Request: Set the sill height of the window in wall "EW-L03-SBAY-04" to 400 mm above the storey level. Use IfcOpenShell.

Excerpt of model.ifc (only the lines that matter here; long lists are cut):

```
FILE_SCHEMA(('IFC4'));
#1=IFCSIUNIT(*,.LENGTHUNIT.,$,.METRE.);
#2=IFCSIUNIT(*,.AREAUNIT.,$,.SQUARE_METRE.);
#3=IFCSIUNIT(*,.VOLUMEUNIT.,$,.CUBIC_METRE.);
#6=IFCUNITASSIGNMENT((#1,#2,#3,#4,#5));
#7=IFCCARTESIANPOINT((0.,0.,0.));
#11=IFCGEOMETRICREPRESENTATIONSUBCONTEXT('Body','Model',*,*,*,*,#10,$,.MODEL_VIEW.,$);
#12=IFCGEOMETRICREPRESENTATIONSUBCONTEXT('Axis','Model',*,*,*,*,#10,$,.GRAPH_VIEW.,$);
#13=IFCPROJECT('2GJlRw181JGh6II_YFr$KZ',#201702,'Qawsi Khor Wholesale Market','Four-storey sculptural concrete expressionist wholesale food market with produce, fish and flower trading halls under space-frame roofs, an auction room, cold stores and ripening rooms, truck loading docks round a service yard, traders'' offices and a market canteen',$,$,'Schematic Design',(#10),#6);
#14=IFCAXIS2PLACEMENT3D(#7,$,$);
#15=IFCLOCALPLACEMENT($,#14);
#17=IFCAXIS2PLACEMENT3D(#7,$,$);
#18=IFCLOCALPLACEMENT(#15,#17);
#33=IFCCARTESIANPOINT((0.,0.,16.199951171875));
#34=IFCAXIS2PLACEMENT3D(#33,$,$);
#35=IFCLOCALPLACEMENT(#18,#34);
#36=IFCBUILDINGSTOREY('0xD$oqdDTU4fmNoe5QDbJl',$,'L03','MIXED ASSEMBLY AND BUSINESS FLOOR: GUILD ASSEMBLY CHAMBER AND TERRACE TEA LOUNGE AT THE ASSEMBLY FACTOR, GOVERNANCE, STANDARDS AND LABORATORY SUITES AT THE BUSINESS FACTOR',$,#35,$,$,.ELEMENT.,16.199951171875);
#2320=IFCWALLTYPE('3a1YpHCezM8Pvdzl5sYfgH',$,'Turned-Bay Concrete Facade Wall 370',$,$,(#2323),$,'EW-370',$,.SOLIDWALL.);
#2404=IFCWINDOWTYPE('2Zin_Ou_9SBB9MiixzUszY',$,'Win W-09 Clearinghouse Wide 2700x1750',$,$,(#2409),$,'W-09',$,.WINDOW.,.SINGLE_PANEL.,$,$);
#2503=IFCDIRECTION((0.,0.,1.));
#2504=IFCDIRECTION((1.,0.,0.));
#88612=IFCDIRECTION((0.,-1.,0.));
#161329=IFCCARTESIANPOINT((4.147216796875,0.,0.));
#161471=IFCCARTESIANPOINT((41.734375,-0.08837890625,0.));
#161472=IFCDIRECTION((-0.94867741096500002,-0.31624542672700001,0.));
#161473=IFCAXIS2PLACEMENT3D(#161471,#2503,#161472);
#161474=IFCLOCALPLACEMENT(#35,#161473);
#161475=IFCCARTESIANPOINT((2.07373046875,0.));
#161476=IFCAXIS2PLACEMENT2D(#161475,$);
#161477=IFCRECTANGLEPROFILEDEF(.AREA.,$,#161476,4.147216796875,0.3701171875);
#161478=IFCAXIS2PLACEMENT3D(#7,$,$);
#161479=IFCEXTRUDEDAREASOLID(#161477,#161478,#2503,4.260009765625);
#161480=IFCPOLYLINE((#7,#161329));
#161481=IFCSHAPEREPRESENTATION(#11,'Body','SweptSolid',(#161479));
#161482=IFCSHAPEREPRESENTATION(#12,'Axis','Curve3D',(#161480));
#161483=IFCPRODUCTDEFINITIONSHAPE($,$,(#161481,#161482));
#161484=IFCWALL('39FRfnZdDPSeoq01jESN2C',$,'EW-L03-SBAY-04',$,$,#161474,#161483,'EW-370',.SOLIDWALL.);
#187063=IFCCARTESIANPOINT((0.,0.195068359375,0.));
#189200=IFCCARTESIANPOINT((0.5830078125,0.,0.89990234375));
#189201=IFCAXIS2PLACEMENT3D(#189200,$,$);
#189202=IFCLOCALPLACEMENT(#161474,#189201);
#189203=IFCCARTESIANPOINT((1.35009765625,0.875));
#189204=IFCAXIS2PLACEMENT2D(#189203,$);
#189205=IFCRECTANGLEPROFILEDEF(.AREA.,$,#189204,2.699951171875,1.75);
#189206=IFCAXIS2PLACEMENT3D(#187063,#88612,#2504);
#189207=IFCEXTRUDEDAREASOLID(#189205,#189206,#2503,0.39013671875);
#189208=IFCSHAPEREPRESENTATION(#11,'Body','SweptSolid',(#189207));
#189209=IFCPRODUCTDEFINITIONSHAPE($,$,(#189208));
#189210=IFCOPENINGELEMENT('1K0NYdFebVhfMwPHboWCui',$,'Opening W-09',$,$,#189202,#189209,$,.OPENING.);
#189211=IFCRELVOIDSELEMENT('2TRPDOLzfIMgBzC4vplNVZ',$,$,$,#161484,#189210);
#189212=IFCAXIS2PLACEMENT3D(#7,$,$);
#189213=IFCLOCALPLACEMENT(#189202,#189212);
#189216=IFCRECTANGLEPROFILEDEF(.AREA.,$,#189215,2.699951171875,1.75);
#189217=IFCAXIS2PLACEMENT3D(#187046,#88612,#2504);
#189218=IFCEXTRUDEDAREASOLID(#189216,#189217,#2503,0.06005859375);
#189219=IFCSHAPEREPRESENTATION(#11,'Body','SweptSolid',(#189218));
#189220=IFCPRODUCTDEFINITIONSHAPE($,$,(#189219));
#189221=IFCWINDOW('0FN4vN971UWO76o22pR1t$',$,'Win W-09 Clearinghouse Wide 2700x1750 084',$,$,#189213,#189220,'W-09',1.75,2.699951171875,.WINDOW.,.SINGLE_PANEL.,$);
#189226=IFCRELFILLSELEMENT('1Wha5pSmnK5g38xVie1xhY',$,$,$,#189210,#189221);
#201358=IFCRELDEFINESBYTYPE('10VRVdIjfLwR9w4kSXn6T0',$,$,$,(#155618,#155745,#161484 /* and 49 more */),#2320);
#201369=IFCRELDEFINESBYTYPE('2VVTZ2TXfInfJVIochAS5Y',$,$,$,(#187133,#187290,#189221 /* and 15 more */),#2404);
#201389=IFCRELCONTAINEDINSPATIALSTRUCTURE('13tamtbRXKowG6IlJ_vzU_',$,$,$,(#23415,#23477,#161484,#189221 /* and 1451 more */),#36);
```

```python
import numpy as np
import ifcopenshell
import ifcopenshell.api.geometry
import ifcopenshell.geom
import ifcopenshell.util.element
import ifcopenshell.util.placement
import ifcopenshell.util.shape
import ifcopenshell.util.unit

model = ifcopenshell.open("model.ifc")
unit_scale = ifcopenshell.util.unit.calculate_unit_scale(model)

window = model.by_guid("0FN4vN971UWO76o22pR1t$")
opening = window.FillsVoids[0].RelatingOpeningElement
storey = ifcopenshell.util.element.get_container(window, ifc_class="IfcBuildingStorey")
level = ifcopenshell.util.placement.get_local_placement(storey.ObjectPlacement)[2, 3]

# The opening's origin need not be at the sill, so measure its lowest point.
shape = ifcopenshell.geom.create_shape(ifcopenshell.geom.settings(), opening)
bottom = ifcopenshell.util.shape.get_shape_bottom_elevation(shape, shape.geometry) / unit_scale
dz = level + 0.4 / unit_scale - bottom

shift = np.array([0.0, 0.0, dz])
# The window is placed relative to its opening, so it follows when the opening moves.
matrix = ifcopenshell.util.placement.get_local_placement(opening.ObjectPlacement)
matrix[:3, 3] += shift
ifcopenshell.api.geometry.edit_object_placement(
    model, product=opening, matrix=matrix, is_si=False, should_transform_children=True
)

print(f"moved by {dz * unit_scale:+.3f} m")

model.write("model_rev.ifc")
```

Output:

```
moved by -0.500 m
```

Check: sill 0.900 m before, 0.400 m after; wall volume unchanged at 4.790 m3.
